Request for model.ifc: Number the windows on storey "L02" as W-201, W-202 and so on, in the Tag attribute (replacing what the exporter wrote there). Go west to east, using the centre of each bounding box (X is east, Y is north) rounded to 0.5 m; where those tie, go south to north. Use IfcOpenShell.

First a look at what the model holds.

```python
import ifcopenshell
import ifcopenshell.util.element
import ifcopenshell.util.placement

model = ifcopenshell.open("model.ifc")
print(model.schema)
storey = next(s for s in model.by_type("IfcBuildingStorey") if s.Name == "L02")
windows = [e for e in ifcopenshell.util.element.get_decomposition(storey) if e.is_a("IfcWindow")]
for e in sorted(windows, key=lambda e: e.id()):
    origin = ifcopenshell.util.placement.get_local_placement(e.ObjectPlacement)[:3, 3]
    print(e.id(), e.Tag, e.Name, origin.round(2) + 0.0, sep=" | ")
```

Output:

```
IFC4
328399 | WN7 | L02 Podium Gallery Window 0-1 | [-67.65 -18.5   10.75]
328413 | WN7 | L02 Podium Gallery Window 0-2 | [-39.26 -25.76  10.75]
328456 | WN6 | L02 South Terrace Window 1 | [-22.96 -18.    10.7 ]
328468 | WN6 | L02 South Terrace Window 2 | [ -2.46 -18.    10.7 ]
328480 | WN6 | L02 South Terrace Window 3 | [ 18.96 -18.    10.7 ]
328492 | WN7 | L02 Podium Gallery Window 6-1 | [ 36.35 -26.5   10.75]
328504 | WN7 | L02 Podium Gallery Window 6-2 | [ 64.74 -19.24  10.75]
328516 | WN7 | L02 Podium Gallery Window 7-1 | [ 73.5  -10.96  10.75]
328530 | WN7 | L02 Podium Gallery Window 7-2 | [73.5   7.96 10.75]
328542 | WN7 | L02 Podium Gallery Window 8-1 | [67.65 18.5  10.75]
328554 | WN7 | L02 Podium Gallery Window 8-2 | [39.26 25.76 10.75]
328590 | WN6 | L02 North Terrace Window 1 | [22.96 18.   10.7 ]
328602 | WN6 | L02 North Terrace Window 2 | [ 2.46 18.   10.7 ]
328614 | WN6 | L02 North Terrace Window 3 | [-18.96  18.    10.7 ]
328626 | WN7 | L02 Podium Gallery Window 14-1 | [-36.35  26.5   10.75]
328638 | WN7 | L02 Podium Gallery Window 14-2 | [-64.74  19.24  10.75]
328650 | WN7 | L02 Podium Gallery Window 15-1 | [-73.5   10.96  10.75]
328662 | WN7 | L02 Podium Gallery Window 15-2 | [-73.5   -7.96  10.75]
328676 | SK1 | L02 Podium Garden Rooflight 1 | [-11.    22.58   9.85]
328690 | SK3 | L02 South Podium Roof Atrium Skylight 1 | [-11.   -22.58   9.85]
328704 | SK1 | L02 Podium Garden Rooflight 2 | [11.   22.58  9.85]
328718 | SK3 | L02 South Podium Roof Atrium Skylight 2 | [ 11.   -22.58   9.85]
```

```python
import ifcopenshell
import ifcopenshell.geom
import ifcopenshell.util.element
import ifcopenshell.util.shape

model = ifcopenshell.open("model.ifc")
settings = ifcopenshell.geom.settings()
settings.set("use-world-coords", True)


def centre(element):
    shape = ifcopenshell.geom.create_shape(settings, element)
    return ifcopenshell.util.shape.get_bbox_centroid(shape.geometry)


storey = next(s for s in model.by_type("IfcBuildingStorey") if s.Name == "L02")
windows = [e for e in ifcopenshell.util.element.get_decomposition(storey) if e.is_a("IfcWindow")]

# Insertion points can sit at a corner or the storey origin, so sort by the geometry (in metres).
centres = {e: centre(e) for e in windows}
windows.sort(key=lambda e: (round(centres[e][0] / 0.5), centres[e][1]))

for i, e in enumerate(windows, start=1):
    number = f"W-2{i:02d}"
    e.Tag = number
    print(e.id(), number)

model.write("model-out.ifc")
```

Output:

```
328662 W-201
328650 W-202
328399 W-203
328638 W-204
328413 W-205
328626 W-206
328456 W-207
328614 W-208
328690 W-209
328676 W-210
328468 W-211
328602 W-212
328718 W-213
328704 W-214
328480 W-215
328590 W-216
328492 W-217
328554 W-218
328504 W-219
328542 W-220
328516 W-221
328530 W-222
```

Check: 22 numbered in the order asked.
